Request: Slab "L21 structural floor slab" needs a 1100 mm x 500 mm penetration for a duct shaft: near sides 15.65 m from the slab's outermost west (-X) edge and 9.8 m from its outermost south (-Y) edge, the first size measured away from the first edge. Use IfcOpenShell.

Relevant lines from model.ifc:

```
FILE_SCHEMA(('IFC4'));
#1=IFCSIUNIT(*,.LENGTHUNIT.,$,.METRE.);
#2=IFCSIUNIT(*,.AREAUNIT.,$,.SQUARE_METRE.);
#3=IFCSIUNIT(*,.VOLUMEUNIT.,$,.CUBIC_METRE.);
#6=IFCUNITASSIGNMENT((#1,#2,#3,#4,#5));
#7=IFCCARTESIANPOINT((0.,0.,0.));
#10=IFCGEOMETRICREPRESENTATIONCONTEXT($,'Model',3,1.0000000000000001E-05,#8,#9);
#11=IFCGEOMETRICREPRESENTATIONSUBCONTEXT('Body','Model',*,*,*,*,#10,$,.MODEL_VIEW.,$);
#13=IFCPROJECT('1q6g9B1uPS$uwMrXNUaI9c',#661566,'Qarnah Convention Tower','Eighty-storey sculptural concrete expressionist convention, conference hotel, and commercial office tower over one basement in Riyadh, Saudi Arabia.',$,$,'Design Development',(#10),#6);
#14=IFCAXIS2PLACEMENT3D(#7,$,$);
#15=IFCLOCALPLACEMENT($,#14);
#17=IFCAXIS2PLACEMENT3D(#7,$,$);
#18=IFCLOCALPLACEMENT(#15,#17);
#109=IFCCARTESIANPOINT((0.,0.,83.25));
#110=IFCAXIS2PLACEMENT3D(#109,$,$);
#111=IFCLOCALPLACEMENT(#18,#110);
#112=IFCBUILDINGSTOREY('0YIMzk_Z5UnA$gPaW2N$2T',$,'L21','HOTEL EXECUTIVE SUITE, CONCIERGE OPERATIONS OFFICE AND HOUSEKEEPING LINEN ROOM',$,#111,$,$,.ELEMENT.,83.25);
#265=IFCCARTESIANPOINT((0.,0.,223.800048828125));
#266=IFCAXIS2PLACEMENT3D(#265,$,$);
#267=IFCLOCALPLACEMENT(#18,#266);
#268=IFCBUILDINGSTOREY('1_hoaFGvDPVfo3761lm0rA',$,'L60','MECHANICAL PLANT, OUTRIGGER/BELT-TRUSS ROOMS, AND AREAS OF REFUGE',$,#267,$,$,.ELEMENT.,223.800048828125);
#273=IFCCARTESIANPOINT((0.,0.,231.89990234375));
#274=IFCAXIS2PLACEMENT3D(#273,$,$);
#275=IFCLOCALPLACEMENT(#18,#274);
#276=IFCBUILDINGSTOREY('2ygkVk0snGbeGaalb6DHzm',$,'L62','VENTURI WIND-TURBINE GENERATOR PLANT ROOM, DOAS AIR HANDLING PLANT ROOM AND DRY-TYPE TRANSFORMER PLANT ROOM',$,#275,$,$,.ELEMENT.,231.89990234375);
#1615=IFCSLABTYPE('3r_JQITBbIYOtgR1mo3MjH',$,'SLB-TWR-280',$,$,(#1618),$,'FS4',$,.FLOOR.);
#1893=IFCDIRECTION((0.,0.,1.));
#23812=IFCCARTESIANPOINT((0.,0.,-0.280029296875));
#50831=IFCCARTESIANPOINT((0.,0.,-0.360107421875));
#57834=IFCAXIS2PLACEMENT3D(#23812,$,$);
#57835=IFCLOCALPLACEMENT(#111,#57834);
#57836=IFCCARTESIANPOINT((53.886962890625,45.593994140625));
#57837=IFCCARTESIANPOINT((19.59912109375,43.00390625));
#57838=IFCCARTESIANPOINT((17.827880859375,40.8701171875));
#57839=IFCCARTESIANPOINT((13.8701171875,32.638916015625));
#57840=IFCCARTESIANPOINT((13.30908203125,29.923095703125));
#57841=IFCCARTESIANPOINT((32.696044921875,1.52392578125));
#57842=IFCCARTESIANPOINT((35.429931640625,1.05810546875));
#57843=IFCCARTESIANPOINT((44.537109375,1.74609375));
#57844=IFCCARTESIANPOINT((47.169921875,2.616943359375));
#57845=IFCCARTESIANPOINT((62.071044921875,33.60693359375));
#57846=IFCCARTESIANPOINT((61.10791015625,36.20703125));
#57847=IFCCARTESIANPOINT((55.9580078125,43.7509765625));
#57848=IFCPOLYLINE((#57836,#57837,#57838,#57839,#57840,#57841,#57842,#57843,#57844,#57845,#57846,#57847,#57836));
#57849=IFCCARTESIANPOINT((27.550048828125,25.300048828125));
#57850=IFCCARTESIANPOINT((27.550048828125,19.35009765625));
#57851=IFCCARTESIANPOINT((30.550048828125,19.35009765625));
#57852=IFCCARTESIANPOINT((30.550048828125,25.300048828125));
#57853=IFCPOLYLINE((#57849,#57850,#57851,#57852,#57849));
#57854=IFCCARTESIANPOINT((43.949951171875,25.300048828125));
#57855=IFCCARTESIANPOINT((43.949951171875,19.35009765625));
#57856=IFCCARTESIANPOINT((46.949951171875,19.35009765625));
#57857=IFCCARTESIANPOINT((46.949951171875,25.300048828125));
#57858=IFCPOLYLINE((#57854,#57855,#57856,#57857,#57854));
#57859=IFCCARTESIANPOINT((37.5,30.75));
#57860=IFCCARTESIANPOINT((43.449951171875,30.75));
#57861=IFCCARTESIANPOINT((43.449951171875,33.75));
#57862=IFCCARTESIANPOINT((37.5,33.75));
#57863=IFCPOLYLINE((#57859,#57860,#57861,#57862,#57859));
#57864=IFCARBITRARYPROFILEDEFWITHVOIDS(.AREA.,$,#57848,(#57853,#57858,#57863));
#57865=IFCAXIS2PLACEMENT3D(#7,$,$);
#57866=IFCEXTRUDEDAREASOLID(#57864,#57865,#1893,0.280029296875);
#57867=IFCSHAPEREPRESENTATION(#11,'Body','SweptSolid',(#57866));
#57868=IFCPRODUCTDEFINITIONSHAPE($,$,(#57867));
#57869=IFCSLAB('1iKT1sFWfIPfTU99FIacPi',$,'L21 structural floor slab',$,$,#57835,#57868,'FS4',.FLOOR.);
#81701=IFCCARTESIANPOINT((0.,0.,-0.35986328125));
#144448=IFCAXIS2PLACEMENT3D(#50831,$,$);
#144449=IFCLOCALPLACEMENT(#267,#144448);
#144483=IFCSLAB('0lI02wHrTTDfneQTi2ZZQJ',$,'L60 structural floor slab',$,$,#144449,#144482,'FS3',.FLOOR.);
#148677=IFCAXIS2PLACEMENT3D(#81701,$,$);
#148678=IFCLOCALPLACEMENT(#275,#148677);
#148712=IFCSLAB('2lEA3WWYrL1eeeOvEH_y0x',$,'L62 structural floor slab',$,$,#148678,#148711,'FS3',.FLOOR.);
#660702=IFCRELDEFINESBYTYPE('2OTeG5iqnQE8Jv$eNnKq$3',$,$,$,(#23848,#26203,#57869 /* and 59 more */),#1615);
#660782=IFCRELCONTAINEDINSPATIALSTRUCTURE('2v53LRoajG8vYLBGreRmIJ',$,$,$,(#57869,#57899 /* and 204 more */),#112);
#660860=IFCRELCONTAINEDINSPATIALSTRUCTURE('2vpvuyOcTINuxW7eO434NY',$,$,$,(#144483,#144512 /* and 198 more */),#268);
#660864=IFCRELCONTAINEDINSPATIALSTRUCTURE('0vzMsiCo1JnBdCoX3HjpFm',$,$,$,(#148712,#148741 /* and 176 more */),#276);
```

```python
import numpy as np
import ifcopenshell
import ifcopenshell.api.feature
import ifcopenshell.api.geometry
import ifcopenshell.api.root
import ifcopenshell.geom
import ifcopenshell.util.placement
import ifcopenshell.util.representation
import ifcopenshell.util.shape
import ifcopenshell.util.unit

model = ifcopenshell.open("model.ifc")
unit_scale = ifcopenshell.util.unit.calculate_unit_scale(model)
settings = ifcopenshell.geom.settings()


def volume(element):
    """Net volume in cubic metres, openings subtracted."""
    shape = ifcopenshell.geom.create_shape(settings, element)
    return ifcopenshell.util.shape.get_volume(shape.geometry)


slab = model.by_id(57869)
before = volume(slab)

# Extent in the slab's own axes, in metres. The edges named are its -X and -Y sides.
slab_shape = ifcopenshell.geom.create_shape(settings, slab)
vertices = ifcopenshell.util.shape.get_vertices(slab_shape.geometry)
x_min, y_min, bottom = vertices.min(axis=0)
top = vertices[:, 2].max()

opening = ifcopenshell.api.root.create_entity(model, ifc_class="IfcOpeningElement", name="Duct shaft opening", predefined_type="OPENING")
context = ifcopenshell.util.representation.get_context(model, "Model", "Body", "MODEL_VIEW")
width, depth = 1.1, 0.5
outline = [(0.0, 0.0), (width, 0.0), (width, depth), (0.0, depth), (0.0, 0.0)]
# Overshoot both faces by 50 mm so the cut is clean.
shape = ifcopenshell.api.geometry.add_slab_representation(
    model, context=context, depth=top - bottom + 0.1, polyline=outline
)
ifcopenshell.api.geometry.assign_representation(model, product=opening, representation=shape)

matrix = ifcopenshell.util.placement.get_local_placement(slab.ObjectPlacement)
matrix[:, 3] = matrix @ np.append(np.array([x_min + 15.65, y_min + 9.8, bottom - 0.05]) / unit_scale, 1.0)
ifcopenshell.api.geometry.edit_object_placement(model, product=opening, matrix=matrix, is_si=False)
ifcopenshell.api.feature.add_feature(model, feature=opening, element=slab)

after = volume(slab)

print(f"slab volume {before:.3f} -> {after:.3f} m3")

model.write("model_edited.ifc")
```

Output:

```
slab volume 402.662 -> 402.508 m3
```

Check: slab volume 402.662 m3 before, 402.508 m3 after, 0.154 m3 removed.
